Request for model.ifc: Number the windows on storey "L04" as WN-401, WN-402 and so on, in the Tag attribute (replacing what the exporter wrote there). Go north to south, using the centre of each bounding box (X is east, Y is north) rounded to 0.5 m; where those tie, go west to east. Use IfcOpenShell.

First a look at what the model holds.

```python
import ifcopenshell
import ifcopenshell.util.element
import ifcopenshell.util.placement

model = ifcopenshell.open("model.ifc")
print(model.schema)
storey = next(s for s in model.by_type("IfcBuildingStorey") if s.Name == "L04")
windows = [e for e in ifcopenshell.util.element.get_decomposition(storey) if e.is_a("IfcWindow")]
for e in sorted(windows, key=lambda e: e.id()):
    origin = ifcopenshell.util.placement.get_local_placement(e.ObjectPlacement)[:3, 3]
    print(e.id(), e.Tag, e.Name, origin.round(2) + 0.0, sep=" | ")
```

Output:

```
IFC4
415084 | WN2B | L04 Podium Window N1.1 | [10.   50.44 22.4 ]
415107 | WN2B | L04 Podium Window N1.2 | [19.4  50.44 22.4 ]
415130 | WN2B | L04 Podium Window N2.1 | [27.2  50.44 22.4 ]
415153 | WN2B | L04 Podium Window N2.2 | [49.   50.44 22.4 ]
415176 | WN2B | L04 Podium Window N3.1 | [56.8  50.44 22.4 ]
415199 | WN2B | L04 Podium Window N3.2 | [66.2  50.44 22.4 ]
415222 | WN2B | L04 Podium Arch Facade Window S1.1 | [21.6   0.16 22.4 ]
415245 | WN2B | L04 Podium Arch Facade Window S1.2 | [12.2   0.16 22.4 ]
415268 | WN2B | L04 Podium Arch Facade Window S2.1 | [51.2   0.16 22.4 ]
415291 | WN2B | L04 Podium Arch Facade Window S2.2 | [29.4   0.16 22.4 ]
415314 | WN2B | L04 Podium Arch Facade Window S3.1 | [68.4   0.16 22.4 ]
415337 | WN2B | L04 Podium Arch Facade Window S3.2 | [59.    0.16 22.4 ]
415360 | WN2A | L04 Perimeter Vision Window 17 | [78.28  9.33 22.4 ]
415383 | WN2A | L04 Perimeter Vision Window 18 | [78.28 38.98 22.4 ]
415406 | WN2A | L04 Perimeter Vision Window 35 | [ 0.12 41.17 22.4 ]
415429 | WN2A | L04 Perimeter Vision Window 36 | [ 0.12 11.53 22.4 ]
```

```python
import ifcopenshell
import ifcopenshell.geom
import ifcopenshell.util.element
import ifcopenshell.util.shape

model = ifcopenshell.open("model.ifc")
settings = ifcopenshell.geom.settings()
settings.set("use-world-coords", True)


def centre(element):
    shape = ifcopenshell.geom.create_shape(settings, element)
    return ifcopenshell.util.shape.get_bbox_centroid(shape.geometry)


storey = next(s for s in model.by_type("IfcBuildingStorey") if s.Name == "L04")
windows = [e for e in ifcopenshell.util.element.get_decomposition(storey) if e.is_a("IfcWindow")]

# Insertion points can sit at a corner or the storey origin, so sort by the geometry (in metres).
centres = {e: centre(e) for e in windows}
windows.sort(key=lambda e: (-round(centres[e][1] / 0.5), centres[e][0]))

for i, e in enumerate(windows, start=1):
    number = f"WN-4{i:02d}"
    e.Tag = number
    print(e.id(), number)

model.write("model_v2.ifc")
```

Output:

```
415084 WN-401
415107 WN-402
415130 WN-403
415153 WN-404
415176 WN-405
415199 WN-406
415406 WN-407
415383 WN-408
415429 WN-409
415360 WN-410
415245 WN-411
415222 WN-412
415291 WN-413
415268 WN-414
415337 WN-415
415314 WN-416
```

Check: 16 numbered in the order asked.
